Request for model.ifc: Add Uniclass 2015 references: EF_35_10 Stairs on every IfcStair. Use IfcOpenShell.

First a look at what the model holds.

```python
import ifcopenshell

model = ifcopenshell.open("model.ifc")
print(model.schema)
print("classifications:", [c.Name for c in model.by_type("IfcClassification")])
for ifc_class in ("IfcDoor", "IfcRoof", "IfcStair", "IfcWall", "IfcWindow"):
    print(ifc_class, len(model.by_type(ifc_class)))
```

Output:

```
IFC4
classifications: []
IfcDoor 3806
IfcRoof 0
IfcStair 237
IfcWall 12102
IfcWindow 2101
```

```python
import ifcopenshell
import ifcopenshell.api.classification

model = ifcopenshell.open("model.ifc")

system = ifcopenshell.api.classification.add_classification(model, classification="Uniclass 2015")

codes = {
    "IfcStair": ("EF_35_10", "Stairs"),
}
for ifc_class, (code, name) in codes.items():
    products = model.by_type(ifc_class)
    ifcopenshell.api.classification.add_reference(
        model, products=products, classification=system, identification=code, name=name
    )
    print(code, len(products))

model.write("model_rev.ifc")
```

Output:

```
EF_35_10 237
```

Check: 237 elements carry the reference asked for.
